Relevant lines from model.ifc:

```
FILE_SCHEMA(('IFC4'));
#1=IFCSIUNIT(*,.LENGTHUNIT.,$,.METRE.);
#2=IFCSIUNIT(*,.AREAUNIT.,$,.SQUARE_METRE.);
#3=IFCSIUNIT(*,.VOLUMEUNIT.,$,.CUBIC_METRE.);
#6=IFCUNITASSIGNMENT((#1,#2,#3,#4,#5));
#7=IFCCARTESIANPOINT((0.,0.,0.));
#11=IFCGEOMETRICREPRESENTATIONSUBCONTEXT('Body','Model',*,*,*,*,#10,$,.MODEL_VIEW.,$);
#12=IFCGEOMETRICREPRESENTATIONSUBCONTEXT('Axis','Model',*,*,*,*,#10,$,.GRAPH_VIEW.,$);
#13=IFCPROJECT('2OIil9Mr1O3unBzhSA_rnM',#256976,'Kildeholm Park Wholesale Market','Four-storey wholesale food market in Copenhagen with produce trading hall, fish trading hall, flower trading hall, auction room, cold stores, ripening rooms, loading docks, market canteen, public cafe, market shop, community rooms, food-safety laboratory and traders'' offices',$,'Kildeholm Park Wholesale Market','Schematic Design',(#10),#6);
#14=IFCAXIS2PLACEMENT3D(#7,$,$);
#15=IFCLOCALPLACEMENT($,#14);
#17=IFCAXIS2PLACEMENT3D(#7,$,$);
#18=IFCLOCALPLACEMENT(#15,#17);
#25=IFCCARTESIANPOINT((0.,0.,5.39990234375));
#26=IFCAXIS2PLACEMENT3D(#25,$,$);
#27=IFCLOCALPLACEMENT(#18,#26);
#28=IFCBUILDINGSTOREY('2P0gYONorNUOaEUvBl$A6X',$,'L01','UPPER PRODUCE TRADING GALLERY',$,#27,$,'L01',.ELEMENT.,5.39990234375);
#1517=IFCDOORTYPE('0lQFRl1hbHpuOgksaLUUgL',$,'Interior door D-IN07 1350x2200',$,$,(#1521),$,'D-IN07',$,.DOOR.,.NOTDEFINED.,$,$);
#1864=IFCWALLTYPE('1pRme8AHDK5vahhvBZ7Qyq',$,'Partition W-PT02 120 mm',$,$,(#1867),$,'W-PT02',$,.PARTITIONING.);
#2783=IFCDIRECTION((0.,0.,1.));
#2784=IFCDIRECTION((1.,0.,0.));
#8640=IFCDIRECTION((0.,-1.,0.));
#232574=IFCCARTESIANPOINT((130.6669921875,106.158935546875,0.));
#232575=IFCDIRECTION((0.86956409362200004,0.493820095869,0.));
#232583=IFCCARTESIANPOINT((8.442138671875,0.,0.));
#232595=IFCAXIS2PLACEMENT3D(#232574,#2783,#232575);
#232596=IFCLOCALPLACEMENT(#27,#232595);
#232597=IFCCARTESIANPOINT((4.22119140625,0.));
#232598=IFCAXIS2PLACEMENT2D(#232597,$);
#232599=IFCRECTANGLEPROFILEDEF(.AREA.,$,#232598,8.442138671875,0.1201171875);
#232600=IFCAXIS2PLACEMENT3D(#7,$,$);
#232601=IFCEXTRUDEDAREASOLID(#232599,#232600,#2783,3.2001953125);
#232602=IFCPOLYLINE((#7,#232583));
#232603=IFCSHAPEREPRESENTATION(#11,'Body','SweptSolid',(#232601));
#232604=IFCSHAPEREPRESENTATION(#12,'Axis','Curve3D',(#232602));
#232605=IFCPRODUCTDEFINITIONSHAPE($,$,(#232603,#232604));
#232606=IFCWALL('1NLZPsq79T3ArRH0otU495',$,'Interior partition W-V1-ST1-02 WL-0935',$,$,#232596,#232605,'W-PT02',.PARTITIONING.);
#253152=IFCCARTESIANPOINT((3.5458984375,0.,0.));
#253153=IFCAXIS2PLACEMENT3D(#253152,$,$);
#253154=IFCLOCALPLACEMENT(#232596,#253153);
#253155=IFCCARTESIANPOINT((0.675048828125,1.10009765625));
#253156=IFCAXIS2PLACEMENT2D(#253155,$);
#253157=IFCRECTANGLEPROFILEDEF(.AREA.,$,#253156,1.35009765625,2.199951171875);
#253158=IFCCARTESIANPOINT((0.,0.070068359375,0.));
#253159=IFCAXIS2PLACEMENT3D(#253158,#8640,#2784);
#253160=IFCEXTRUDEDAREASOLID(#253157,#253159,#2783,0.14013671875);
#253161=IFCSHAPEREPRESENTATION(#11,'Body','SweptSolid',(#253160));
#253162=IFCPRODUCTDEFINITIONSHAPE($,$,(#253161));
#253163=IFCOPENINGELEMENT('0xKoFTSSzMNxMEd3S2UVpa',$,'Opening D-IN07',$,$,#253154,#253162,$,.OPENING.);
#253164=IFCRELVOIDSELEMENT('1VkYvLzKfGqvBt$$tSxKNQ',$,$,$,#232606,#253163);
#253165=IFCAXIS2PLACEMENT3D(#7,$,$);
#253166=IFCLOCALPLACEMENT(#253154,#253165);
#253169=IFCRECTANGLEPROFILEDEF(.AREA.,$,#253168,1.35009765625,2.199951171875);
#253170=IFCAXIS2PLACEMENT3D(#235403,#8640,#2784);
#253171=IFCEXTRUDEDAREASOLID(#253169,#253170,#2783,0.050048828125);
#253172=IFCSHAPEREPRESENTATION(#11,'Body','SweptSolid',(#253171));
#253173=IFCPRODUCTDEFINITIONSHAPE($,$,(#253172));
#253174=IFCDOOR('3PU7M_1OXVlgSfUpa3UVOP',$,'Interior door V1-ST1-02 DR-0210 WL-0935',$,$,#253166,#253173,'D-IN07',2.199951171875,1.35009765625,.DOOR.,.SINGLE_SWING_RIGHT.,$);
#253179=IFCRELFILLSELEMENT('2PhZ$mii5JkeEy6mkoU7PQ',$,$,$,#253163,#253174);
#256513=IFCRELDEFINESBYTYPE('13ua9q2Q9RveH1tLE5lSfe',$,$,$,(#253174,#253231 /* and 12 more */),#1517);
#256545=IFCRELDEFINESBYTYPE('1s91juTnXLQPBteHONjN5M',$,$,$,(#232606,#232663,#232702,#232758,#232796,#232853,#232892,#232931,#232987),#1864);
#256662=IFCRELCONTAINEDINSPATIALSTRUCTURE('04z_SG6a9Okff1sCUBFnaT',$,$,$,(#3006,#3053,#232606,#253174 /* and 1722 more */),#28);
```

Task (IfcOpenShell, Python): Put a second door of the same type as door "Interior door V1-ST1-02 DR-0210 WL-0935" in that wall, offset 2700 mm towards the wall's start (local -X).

```python
import ifcopenshell
import ifcopenshell.api.feature
import ifcopenshell.api.geometry
import ifcopenshell.api.root
import ifcopenshell.geom
import ifcopenshell.util.element
import ifcopenshell.util.placement
import ifcopenshell.util.shape

model = ifcopenshell.open("model.ifc")
settings = ifcopenshell.geom.settings()


def volume(element):
    """Net volume in cubic metres, openings subtracted."""
    shape = ifcopenshell.geom.create_shape(settings, element)
    return ifcopenshell.util.shape.get_volume(shape.geometry)


door = model.by_id(253174)
opening = door.FillsVoids[0].RelatingOpeningElement
wall = opening.VoidsElements[0].RelatingBuildingElement
before = volume(wall)
shift = ifcopenshell.util.placement.get_local_placement(wall.ObjectPlacement)[:3, 0] * -2.7

# copy_class copies the void relationship, type, container and properties, but no geometry.
new_opening = ifcopenshell.api.root.copy_class(model, product=opening)
new_opening.Representation = ifcopenshell.util.element.copy_deep(
    model, opening.Representation, exclude=["IfcGeometricRepresentationContext", "IfcRepresentationMap"]
)
new_door = ifcopenshell.api.root.copy_class(model, product=door)
new_door.Representation = ifcopenshell.util.element.copy_deep(
    model, door.Representation, exclude=["IfcGeometricRepresentationContext", "IfcRepresentationMap"]
)
new_door.Tag = None
ifcopenshell.api.feature.add_filling(model, opening=new_opening, element=new_door)

for old, new in ((opening, new_opening), (door, new_door)):
    matrix = ifcopenshell.util.placement.get_local_placement(old.ObjectPlacement)
    matrix[:3, 3] += shift
    ifcopenshell.api.geometry.edit_object_placement(model, product=new, matrix=matrix, is_si=False)

after = volume(wall)

print(f"wall volume {before:.3f} -> {after:.3f} m3")

model.write("model_v2.ifc")
```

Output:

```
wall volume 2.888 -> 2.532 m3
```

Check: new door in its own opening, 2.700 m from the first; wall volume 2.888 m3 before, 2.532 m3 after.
